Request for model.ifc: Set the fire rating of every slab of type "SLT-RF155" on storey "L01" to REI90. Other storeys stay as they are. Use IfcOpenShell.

First a look at what the model holds.

```python
import ifcopenshell
import ifcopenshell.util.element

model = ifcopenshell.open("model.ifc")
print(model.schema)
storey = next(s for s in model.by_type("IfcBuildingStorey") if s.Name == "L01")
slabs = [e for e in ifcopenshell.util.element.get_decomposition(storey) if e.is_a("IfcSlab")]
seen = {}
for e in slabs:
    element_type = ifcopenshell.util.element.get_type(e)
    key = (element_type.Name if element_type != e and element_type else None, ifcopenshell.util.element.get_pset(e, "Pset_SlabCommon", "FireRating"))
    seen[key] = seen.get(key, 0) + 1
for (name, value), count in sorted(seen.items(), key=str):
    print(count, "x", name, "|", value)
```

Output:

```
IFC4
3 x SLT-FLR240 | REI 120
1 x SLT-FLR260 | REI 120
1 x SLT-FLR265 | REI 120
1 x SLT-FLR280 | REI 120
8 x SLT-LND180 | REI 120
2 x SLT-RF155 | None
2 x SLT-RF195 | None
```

```python
import ifcopenshell
import ifcopenshell.api.pset
import ifcopenshell.util.element

model = ifcopenshell.open("model.ifc")

storey = next(s for s in model.by_type("IfcBuildingStorey") if s.Name == "L01")
slabs = [e for e in ifcopenshell.util.element.get_decomposition(storey) if e.is_a("IfcSlab")]

count = 0
for e in slabs:
    element_type = ifcopenshell.util.element.get_type(e)
    if element_type in (None, e) or element_type.Name != "SLT-RF155":
        continue
    # add_pset returns the element's existing set when there is one.
    pset = ifcopenshell.api.pset.add_pset(model, product=e, name="Pset_SlabCommon")
    ifcopenshell.api.pset.edit_pset(model, pset=pset, properties={"FireRating": "REI90"})
    count += 1

print(count, "slabs updated")

model.write("model_edited.ifc")
```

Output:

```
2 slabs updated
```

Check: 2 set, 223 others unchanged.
